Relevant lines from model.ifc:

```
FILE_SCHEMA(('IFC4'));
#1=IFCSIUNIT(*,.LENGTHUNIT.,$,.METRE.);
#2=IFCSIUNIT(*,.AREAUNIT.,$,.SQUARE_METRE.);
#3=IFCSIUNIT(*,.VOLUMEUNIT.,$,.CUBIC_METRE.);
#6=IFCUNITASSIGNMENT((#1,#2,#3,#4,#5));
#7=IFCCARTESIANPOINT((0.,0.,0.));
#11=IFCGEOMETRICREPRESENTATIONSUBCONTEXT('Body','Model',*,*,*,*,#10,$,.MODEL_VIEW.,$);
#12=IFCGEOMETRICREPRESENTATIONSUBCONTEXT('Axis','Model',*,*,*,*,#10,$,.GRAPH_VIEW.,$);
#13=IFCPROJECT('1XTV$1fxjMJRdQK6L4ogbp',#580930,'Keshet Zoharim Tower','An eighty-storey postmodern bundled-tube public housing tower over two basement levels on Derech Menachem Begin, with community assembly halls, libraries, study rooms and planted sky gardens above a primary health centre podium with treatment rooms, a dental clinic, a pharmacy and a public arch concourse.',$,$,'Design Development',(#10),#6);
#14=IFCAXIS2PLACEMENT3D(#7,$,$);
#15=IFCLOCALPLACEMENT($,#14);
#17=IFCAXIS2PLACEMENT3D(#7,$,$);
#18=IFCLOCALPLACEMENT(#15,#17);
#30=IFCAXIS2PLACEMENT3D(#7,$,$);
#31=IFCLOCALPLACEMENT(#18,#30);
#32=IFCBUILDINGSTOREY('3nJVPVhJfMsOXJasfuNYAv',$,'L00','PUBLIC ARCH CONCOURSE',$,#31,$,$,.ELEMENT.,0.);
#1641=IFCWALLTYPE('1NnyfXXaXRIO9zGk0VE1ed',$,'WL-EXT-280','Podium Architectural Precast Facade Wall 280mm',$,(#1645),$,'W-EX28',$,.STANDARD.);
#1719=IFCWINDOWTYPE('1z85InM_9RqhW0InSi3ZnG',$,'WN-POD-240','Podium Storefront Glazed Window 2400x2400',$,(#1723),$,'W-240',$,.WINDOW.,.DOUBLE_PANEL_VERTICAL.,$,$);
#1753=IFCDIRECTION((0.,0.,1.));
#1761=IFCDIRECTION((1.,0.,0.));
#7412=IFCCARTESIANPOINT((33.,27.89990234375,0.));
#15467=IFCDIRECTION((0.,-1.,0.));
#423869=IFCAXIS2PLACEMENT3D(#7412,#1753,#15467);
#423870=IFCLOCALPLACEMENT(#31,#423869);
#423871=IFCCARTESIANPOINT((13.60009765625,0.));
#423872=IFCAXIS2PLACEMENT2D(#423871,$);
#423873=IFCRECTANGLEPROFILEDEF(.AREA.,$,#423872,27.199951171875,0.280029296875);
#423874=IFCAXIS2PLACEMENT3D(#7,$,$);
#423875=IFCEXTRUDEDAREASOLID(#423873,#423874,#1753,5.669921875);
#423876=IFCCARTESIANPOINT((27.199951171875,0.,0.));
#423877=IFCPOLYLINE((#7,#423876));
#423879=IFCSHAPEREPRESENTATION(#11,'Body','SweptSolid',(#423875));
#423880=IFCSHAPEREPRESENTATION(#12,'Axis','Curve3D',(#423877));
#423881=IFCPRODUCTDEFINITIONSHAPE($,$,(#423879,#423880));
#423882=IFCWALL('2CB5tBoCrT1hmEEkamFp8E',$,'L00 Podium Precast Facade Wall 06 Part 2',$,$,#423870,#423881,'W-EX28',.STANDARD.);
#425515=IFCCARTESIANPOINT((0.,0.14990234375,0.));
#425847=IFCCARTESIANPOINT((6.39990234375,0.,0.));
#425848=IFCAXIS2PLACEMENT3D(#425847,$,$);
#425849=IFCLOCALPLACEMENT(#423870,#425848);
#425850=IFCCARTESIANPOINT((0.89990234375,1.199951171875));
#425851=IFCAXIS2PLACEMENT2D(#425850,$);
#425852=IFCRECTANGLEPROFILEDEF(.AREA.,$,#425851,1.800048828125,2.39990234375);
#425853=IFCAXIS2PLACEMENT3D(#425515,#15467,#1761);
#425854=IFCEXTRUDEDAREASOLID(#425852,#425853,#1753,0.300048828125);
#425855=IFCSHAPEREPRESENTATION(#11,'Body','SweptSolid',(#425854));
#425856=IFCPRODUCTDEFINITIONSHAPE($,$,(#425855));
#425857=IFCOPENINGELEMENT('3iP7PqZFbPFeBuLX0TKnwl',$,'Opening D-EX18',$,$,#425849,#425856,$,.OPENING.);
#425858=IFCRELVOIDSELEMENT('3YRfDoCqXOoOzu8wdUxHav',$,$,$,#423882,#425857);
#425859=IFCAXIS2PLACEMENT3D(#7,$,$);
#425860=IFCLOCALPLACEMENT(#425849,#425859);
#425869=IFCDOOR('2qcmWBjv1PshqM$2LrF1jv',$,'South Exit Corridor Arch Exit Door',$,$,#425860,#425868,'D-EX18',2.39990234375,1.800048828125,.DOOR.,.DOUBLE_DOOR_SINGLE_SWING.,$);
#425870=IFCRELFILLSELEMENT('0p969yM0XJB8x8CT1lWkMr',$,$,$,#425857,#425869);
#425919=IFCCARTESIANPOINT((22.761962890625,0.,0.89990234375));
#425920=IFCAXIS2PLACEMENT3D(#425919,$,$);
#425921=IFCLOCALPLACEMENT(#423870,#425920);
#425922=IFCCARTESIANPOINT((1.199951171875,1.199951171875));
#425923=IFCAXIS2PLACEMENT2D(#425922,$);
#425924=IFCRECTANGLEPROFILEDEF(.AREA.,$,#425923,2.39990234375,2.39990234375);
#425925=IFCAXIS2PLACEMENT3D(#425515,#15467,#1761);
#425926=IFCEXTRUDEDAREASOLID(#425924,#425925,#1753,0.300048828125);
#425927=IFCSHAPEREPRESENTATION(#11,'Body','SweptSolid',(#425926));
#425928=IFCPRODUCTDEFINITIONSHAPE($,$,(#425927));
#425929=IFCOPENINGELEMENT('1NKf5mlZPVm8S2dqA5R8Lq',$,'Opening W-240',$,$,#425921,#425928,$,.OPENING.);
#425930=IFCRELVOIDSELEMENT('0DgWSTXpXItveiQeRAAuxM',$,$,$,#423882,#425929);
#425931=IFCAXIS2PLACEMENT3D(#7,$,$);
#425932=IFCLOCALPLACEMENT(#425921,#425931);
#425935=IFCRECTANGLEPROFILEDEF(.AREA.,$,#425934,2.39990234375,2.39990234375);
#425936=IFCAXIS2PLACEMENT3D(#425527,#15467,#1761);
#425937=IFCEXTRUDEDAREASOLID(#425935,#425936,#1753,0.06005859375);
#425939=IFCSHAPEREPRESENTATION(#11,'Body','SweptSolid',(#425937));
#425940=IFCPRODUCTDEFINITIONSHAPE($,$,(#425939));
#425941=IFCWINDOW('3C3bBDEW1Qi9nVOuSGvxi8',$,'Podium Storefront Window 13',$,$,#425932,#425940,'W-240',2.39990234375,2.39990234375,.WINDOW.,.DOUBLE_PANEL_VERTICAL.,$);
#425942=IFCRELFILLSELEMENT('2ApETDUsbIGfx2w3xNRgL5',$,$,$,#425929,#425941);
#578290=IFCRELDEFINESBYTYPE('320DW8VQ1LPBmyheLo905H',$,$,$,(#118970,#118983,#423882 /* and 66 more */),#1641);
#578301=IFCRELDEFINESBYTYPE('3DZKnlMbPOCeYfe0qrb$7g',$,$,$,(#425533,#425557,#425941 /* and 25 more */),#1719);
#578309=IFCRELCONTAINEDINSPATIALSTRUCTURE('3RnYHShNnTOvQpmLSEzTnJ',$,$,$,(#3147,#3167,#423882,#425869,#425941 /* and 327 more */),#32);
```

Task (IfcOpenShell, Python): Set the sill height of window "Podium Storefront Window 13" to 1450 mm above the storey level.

```python
import numpy as np
import ifcopenshell
import ifcopenshell.api.geometry
import ifcopenshell.geom
import ifcopenshell.util.element
import ifcopenshell.util.placement
import ifcopenshell.util.shape
import ifcopenshell.util.unit

model = ifcopenshell.open("model.ifc")
unit_scale = ifcopenshell.util.unit.calculate_unit_scale(model)

window = model.by_id(425941)
opening = window.FillsVoids[0].RelatingOpeningElement
storey = ifcopenshell.util.element.get_container(window, ifc_class="IfcBuildingStorey")
level = ifcopenshell.util.placement.get_local_placement(storey.ObjectPlacement)[2, 3]

# The opening's origin need not be at the sill, so measure its lowest point.
shape = ifcopenshell.geom.create_shape(ifcopenshell.geom.settings(), opening)
bottom = ifcopenshell.util.shape.get_shape_bottom_elevation(shape, shape.geometry) / unit_scale
dz = level + 1.45 - bottom

shift = np.array([0.0, 0.0, dz])
# The window is placed relative to its opening, so it follows when the opening moves.
matrix = ifcopenshell.util.placement.get_local_placement(opening.ObjectPlacement)
matrix[:3, 3] += shift
ifcopenshell.api.geometry.edit_object_placement(
    model, product=opening, matrix=matrix, is_si=False, should_transform_children=True
)

print(f"moved by {dz * unit_scale:+.3f} m")

model.write("model_v2.ifc")
```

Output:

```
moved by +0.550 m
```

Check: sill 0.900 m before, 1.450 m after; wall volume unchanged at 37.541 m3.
